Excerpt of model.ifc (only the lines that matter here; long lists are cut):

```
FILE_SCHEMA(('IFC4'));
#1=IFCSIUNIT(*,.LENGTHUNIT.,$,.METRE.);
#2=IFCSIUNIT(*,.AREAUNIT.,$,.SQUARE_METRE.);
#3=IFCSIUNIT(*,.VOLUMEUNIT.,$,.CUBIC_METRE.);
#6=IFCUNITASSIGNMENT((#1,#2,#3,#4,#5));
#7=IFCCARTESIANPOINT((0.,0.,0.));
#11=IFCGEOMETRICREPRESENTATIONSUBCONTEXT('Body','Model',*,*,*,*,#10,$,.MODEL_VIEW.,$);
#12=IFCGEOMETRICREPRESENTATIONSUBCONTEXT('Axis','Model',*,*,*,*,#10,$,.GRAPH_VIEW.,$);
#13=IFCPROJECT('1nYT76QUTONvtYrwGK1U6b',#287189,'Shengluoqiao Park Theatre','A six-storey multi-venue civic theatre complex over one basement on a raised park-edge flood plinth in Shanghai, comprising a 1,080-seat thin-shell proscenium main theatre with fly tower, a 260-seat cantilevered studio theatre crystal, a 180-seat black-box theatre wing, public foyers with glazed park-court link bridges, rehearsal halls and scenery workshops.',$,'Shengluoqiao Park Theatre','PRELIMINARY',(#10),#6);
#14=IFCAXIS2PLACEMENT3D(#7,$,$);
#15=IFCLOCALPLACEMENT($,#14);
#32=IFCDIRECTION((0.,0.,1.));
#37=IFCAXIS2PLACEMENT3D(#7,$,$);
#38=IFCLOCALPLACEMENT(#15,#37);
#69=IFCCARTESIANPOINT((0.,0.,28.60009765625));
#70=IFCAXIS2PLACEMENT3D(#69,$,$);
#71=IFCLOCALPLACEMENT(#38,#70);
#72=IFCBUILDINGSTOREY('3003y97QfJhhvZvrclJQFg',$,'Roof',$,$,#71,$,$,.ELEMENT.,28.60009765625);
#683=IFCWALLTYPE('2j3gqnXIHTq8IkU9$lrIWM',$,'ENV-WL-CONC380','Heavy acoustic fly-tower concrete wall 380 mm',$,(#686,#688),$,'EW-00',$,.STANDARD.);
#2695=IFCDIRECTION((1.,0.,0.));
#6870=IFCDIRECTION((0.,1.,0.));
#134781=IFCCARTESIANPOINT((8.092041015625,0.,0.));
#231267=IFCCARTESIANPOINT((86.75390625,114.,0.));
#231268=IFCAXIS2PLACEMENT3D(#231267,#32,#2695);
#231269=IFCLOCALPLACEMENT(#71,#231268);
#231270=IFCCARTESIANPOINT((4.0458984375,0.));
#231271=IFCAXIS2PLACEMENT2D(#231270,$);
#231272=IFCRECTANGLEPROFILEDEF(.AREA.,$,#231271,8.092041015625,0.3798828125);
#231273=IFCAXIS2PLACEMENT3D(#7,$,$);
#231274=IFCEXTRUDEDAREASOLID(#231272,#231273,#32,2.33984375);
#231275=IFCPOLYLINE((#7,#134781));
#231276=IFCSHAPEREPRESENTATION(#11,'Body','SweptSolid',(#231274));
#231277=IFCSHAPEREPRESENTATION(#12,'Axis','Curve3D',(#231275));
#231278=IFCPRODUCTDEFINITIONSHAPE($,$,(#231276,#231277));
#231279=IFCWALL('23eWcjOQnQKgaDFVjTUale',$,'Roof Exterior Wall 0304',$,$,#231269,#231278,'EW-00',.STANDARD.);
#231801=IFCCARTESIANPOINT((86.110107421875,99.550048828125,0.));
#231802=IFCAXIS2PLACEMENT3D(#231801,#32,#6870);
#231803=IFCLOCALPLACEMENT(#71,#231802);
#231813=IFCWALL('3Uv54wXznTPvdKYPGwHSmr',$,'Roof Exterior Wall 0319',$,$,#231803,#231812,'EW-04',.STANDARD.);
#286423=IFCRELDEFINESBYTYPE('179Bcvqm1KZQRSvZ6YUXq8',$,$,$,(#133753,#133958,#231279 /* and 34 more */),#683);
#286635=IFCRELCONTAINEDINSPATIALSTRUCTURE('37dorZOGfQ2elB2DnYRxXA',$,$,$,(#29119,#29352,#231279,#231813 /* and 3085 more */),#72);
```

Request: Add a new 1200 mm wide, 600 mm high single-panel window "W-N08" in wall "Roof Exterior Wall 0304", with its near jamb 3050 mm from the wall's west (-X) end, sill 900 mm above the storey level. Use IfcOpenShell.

```python
import numpy as np
import ifcopenshell
import ifcopenshell.api.feature
import ifcopenshell.api.geometry
import ifcopenshell.api.root
import ifcopenshell.api.spatial
import ifcopenshell.geom
import ifcopenshell.util.element
import ifcopenshell.util.placement
import ifcopenshell.util.representation
import ifcopenshell.util.shape
import ifcopenshell.util.unit

model = ifcopenshell.open("model.ifc")
unit_scale = ifcopenshell.util.unit.calculate_unit_scale(model)
settings = ifcopenshell.geom.settings()


def volume(element):
    """Net volume in cubic metres, openings subtracted."""
    shape = ifcopenshell.geom.create_shape(settings, element)
    return ifcopenshell.util.shape.get_volume(shape.geometry)


wall = model.by_id(231279)
storey = ifcopenshell.util.element.get_container(wall, ifc_class="IfcBuildingStorey")
context = ifcopenshell.util.representation.get_context(model, "Model", "Body", "MODEL_VIEW")
before = volume(wall)

width, height, from_end, sill = 1.2, 0.6, 3.05, 0.9  # metres

# The wall runs along its own X axis, and the end named is its -X end.
wall_shape = ifcopenshell.geom.create_shape(settings, wall)
x, y, z = ifcopenshell.util.shape.get_vertices(wall_shape.geometry).T
start = x.min() + from_end
face, thickness = float(y.min()), float(y.max() - y.min())
wall_matrix = ifcopenshell.util.placement.get_local_placement(wall.ObjectPlacement)
level = ifcopenshell.util.placement.get_local_placement(storey.ObjectPlacement)[2, 3]


def in_wall(x, y):
    """Placement at x, y metres in the wall's axes, at sill height."""
    matrix = wall_matrix.copy()
    matrix[:, 3] = wall_matrix @ np.array([x / unit_scale, y / unit_scale, 0.0, 1.0])
    matrix[2, 3] = level + sill / unit_scale
    return matrix


# Opening: a box that overshoots both wall faces by 50 mm.
opening = ifcopenshell.api.root.create_entity(model, ifc_class="IfcOpeningElement", predefined_type="OPENING")
box = ifcopenshell.api.geometry.add_wall_representation(
    model, context=context, length=width, height=height, thickness=thickness + 0.1
)
ifcopenshell.api.geometry.assign_representation(model, product=opening, representation=box)
ifcopenshell.api.geometry.edit_object_placement(model, product=opening, matrix=in_wall(start, face - 0.05), is_si=False)
ifcopenshell.api.feature.add_feature(model, feature=opening, element=wall)

window = ifcopenshell.api.root.create_entity(model, ifc_class="IfcWindow", name="W-N08", predefined_type="WINDOW")
window.OverallWidth, window.OverallHeight = width / unit_scale, height / unit_scale
window.PartitioningType = "SINGLE_PANEL"
body = ifcopenshell.api.geometry.add_window_representation(
    model,
    context=context,
    overall_width=window.OverallWidth,
    overall_height=window.OverallHeight,
    partition_type="SINGLE_PANEL",
)
ifcopenshell.api.geometry.assign_representation(model, product=window, representation=body)
ifcopenshell.api.spatial.assign_container(model, products=[window], relating_structure=storey)
ifcopenshell.api.feature.add_filling(model, opening=opening, element=window)

# Centre the window in the wall's thickness.
ifcopenshell.api.geometry.edit_object_placement(model, product=window, matrix=in_wall(start, face), is_si=False)
window_shape = ifcopenshell.geom.create_shape(settings, window)
depth = ifcopenshell.util.shape.get_vertices(window_shape.geometry)[:, 1]
offset = face + thickness / 2 - (depth.min() + depth.max()) / 2
ifcopenshell.api.geometry.edit_object_placement(model, product=window, matrix=in_wall(start, offset), is_si=False)

after = volume(wall)

print(f"wall volume {before:.3f} -> {after:.3f} m3")

model.write("model_updated.ifc")
```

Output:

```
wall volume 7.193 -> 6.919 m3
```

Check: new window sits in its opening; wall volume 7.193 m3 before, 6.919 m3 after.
